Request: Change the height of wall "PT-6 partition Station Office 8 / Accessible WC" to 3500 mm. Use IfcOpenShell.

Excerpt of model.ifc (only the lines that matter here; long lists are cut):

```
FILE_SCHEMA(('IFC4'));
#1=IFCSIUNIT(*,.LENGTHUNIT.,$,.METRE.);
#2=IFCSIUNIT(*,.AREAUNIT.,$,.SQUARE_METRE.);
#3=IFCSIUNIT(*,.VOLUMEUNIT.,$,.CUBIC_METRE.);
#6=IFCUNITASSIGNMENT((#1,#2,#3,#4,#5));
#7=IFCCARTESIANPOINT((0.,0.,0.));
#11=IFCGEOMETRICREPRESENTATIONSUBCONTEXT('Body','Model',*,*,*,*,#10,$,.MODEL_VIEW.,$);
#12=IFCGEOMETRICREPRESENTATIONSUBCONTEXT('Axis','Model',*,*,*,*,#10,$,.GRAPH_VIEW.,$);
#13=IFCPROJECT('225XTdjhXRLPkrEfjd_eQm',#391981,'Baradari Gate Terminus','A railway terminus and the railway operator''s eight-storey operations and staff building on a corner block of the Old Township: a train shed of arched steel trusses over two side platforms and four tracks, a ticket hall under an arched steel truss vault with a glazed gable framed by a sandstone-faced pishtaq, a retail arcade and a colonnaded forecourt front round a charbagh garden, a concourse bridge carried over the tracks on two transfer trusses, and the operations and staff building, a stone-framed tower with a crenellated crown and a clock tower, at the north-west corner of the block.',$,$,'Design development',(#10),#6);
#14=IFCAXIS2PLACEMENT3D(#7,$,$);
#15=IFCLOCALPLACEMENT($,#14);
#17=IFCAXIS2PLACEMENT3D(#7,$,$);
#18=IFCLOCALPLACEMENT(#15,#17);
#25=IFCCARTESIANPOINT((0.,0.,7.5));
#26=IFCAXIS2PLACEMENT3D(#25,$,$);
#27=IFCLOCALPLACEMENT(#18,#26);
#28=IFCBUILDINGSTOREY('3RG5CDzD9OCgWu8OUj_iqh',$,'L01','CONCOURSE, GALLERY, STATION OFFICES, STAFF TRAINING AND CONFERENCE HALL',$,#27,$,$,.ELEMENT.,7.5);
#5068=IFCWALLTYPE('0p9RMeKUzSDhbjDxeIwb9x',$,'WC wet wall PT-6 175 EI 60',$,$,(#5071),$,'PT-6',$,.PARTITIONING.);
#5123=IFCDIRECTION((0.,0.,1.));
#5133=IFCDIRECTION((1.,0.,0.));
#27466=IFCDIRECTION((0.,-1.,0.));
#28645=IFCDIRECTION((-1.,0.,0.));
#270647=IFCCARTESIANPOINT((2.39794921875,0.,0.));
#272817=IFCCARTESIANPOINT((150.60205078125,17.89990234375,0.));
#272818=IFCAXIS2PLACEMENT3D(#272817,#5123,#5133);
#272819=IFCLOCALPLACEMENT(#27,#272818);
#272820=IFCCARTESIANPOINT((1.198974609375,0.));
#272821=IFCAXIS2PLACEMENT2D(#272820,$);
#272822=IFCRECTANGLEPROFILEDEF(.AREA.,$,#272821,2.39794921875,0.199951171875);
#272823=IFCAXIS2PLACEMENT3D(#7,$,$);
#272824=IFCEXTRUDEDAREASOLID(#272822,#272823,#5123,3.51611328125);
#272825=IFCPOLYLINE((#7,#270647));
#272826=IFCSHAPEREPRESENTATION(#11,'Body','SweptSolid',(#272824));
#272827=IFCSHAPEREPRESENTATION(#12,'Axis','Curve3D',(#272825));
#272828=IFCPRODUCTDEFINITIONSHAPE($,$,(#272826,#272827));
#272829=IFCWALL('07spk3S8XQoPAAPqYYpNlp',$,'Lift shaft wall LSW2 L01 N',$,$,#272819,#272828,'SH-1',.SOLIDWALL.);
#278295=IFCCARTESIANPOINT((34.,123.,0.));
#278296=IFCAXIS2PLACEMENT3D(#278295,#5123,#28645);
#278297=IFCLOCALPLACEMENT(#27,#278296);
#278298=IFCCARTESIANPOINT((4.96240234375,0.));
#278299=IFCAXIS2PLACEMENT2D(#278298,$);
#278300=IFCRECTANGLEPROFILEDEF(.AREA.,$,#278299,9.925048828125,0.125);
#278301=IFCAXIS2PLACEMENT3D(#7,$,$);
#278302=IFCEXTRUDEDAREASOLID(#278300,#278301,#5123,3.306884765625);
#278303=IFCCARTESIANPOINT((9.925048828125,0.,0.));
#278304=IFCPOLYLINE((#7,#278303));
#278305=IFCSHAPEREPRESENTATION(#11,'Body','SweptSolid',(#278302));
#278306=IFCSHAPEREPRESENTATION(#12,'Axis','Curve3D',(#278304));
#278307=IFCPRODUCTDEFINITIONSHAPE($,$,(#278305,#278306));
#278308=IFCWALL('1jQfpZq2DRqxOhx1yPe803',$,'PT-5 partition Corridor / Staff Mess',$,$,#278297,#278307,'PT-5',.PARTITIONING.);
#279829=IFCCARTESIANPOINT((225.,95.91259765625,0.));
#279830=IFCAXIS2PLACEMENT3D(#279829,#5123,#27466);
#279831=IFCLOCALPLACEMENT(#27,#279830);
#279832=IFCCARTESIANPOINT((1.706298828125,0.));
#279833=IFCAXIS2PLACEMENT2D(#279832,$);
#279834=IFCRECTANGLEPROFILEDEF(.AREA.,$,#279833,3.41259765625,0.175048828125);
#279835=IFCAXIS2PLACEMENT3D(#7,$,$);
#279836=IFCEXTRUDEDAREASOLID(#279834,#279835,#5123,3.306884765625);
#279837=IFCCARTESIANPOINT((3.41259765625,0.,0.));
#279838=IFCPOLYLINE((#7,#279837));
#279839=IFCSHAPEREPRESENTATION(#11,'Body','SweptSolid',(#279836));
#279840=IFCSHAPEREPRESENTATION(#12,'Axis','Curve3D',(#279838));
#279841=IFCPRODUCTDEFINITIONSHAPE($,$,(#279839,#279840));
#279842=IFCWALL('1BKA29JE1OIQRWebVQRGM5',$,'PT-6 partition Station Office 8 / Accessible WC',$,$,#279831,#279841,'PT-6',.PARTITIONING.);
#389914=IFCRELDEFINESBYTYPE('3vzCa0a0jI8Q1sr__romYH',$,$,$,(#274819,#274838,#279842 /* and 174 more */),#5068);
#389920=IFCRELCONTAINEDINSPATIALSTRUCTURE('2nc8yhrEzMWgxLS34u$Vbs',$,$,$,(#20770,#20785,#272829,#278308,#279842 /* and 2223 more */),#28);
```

```python
import ifcopenshell
import ifcopenshell.geom
import ifcopenshell.util.representation
import ifcopenshell.util.shape
import ifcopenshell.util.unit

model = ifcopenshell.open("model.ifc")
unit_scale = ifcopenshell.util.unit.calculate_unit_scale(model)
settings = ifcopenshell.geom.settings()


def volume(element):
    """Net volume in cubic metres, openings subtracted."""
    shape = ifcopenshell.geom.create_shape(settings, element)
    return ifcopenshell.util.shape.get_volume(shape.geometry)


wall = model.by_guid("1BKA29JE1OIQRWebVQRGM5")
before = volume(wall)

body = ifcopenshell.util.representation.get_representation(wall, "Model", "Body")
solid = body.Items[0]
old_height = solid.Depth
solid.Depth = 3.5 / unit_scale
after = volume(wall)

print(f"height {old_height:g} -> {solid.Depth:g}, volume {before:.3f} -> {after:.3f} m3")

model.write("model_v2.ifc")
```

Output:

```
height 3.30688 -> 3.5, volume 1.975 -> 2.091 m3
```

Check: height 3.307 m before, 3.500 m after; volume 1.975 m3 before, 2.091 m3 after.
